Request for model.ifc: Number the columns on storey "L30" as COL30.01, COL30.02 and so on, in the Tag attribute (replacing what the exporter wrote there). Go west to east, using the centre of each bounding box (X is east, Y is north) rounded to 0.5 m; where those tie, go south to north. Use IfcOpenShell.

First a look at what the model holds.

```python
import ifcopenshell
import ifcopenshell.util.element
import ifcopenshell.util.placement

model = ifcopenshell.open("model.ifc")
print(model.schema)
storey = next(s for s in model.by_type("IfcBuildingStorey") if s.Name == "L30")
columns = [e for e in ifcopenshell.util.element.get_decomposition(storey) if e.is_a("IfcColumn")]
for e in sorted(columns, key=lambda e: e.id()):
    origin = ifcopenshell.util.placement.get_local_placement(e.ObjectPlacement)[:3, 3]
    print(e.id(), e.Tag, e.Name, origin.round(2) + 0.0, sep=" | ")
```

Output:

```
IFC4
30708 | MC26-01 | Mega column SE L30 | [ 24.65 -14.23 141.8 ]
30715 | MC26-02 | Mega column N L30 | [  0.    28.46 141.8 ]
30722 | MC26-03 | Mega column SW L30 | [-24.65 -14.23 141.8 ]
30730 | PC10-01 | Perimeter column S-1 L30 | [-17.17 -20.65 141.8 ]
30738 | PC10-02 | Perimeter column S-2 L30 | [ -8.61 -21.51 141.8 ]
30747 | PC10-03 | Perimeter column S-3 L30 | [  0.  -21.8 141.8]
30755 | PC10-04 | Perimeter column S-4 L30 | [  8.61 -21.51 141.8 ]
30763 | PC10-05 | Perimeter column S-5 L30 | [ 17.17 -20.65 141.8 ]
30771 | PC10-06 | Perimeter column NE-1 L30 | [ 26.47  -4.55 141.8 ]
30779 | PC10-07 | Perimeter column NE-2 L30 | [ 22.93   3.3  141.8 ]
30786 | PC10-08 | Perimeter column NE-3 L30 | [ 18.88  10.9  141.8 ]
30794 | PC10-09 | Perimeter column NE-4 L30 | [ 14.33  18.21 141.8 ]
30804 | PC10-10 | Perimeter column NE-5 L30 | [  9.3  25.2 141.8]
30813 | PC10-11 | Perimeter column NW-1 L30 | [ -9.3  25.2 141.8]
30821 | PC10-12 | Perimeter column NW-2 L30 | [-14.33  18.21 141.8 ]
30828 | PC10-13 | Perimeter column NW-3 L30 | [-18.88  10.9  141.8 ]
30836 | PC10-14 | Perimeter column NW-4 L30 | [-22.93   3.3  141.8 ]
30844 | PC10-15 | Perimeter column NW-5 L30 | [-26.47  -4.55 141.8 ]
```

```python
import ifcopenshell
import ifcopenshell.geom
import ifcopenshell.util.element
import ifcopenshell.util.shape

model = ifcopenshell.open("model.ifc")
settings = ifcopenshell.geom.settings()
settings.set("use-world-coords", True)


def centre(element):
    shape = ifcopenshell.geom.create_shape(settings, element)
    return ifcopenshell.util.shape.get_bbox_centroid(shape.geometry)


storey = next(s for s in model.by_type("IfcBuildingStorey") if s.Name == "L30")
columns = [e for e in ifcopenshell.util.element.get_decomposition(storey) if e.is_a("IfcColumn")]

# Insertion points can sit at a corner or the storey origin, so sort by the geometry (in metres).
centres = {e: centre(e) for e in columns}
columns.sort(key=lambda e: (round(centres[e][0] / 0.5), centres[e][1]))

for i, e in enumerate(columns, start=1):
    number = f"COL30.{i:02d}"
    e.Tag = number
    print(e.id(), number)

model.write("model-out.ifc")
```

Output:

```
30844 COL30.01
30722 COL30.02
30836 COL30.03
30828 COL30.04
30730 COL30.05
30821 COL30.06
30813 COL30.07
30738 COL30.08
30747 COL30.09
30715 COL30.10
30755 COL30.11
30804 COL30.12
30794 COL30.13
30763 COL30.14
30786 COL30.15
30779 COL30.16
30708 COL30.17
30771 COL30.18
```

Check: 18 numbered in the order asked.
